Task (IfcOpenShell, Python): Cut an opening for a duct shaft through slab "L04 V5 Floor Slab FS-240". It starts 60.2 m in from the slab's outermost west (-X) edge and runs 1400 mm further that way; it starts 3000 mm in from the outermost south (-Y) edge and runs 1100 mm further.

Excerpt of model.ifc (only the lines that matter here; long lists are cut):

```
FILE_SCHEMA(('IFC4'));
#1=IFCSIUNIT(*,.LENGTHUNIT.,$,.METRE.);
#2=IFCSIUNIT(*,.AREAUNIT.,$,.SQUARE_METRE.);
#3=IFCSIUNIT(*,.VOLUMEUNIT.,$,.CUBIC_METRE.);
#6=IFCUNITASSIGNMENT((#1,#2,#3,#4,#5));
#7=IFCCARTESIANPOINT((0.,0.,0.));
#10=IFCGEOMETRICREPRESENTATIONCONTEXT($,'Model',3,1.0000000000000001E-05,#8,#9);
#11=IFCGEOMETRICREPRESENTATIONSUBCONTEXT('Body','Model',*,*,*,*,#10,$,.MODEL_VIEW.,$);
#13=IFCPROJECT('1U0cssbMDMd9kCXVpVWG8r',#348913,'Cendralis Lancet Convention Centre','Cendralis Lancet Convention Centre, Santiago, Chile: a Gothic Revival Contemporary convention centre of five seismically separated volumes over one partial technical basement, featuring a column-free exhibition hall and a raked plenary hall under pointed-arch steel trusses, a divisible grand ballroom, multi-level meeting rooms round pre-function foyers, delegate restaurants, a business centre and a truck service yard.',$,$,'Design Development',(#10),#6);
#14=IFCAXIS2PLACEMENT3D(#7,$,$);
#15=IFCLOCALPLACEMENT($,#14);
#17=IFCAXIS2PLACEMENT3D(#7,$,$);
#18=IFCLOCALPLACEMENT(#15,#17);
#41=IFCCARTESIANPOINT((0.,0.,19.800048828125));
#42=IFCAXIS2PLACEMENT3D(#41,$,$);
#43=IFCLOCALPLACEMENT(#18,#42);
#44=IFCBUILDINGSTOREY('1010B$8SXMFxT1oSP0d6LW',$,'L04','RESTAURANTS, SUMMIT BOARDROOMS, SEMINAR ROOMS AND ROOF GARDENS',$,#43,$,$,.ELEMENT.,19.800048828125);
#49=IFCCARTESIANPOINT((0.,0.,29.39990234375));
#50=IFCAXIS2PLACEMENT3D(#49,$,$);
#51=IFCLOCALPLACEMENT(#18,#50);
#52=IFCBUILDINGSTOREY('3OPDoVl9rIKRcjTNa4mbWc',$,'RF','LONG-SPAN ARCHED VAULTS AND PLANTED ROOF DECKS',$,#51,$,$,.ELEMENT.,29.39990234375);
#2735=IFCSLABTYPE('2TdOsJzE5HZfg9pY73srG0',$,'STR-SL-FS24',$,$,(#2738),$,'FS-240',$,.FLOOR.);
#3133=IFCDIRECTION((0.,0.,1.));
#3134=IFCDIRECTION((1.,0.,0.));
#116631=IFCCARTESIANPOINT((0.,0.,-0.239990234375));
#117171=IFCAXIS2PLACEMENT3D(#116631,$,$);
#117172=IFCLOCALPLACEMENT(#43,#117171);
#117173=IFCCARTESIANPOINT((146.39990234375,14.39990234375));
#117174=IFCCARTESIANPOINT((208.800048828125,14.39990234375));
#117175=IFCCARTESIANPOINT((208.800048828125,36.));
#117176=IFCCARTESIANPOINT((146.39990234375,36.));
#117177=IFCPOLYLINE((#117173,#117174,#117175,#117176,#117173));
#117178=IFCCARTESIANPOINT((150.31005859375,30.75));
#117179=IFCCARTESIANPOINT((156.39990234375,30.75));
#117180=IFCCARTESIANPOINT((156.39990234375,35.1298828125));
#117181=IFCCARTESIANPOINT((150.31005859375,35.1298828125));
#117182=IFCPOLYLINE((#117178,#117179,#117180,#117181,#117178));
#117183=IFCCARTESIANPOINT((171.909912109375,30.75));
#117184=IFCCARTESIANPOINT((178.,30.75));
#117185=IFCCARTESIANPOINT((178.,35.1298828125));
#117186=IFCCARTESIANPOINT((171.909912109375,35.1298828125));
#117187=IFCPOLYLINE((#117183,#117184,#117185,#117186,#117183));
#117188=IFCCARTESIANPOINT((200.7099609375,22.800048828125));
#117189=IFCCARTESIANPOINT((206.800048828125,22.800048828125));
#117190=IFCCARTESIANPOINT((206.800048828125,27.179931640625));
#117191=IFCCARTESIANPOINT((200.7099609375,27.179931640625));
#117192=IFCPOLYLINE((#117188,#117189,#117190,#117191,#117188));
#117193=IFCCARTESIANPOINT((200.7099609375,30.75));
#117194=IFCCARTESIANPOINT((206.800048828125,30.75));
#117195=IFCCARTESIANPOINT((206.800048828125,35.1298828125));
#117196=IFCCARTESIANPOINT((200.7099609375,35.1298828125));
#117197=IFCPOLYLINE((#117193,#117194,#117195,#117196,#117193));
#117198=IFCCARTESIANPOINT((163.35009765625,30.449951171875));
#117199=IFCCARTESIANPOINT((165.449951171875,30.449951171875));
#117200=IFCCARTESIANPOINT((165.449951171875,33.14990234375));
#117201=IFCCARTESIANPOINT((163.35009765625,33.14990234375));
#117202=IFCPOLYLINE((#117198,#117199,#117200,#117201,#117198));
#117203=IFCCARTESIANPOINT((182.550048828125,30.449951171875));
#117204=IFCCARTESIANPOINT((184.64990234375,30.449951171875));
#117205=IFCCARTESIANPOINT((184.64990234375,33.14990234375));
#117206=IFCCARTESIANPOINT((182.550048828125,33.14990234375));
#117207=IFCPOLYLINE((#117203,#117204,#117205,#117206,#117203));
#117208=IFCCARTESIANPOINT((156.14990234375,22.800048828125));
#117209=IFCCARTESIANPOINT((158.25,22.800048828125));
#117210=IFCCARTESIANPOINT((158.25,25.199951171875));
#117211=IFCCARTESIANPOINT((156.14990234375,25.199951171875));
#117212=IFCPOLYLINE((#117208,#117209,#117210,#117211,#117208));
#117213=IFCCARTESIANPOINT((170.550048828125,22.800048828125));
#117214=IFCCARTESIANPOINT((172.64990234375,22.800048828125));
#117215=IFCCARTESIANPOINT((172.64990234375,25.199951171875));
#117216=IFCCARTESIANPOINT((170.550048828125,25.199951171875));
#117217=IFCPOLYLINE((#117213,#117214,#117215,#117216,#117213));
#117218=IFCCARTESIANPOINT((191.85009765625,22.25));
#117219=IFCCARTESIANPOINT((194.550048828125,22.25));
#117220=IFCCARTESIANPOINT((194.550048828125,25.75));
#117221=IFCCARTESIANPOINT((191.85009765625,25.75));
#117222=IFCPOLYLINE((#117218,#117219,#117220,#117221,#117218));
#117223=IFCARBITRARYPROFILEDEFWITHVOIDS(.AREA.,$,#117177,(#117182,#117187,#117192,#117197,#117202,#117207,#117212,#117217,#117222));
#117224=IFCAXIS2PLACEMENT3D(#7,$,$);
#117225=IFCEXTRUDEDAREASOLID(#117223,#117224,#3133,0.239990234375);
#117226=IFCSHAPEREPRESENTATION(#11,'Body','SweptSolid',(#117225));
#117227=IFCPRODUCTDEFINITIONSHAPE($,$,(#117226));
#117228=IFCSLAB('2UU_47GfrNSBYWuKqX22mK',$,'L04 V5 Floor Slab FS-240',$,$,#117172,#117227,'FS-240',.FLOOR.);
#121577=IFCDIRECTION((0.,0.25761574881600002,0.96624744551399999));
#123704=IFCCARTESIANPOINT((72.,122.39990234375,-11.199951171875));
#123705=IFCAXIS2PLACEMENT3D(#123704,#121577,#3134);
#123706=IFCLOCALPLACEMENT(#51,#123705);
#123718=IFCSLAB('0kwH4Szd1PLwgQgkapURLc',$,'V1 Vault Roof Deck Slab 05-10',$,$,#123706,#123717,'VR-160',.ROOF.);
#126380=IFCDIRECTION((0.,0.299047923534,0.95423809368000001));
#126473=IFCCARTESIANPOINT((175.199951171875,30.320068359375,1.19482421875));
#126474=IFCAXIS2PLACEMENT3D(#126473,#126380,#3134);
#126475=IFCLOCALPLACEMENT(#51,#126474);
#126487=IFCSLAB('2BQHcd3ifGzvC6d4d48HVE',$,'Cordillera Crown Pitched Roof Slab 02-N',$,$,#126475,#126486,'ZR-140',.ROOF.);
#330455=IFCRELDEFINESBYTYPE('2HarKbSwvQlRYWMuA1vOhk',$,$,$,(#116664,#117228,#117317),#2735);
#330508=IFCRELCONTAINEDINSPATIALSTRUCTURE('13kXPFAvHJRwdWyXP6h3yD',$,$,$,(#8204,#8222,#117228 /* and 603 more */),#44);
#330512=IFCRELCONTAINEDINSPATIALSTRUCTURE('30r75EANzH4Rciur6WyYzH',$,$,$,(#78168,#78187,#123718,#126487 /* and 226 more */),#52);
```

```python
import numpy as np
import ifcopenshell
import ifcopenshell.api.feature
import ifcopenshell.api.geometry
import ifcopenshell.api.root
import ifcopenshell.geom
import ifcopenshell.util.placement
import ifcopenshell.util.representation
import ifcopenshell.util.shape
import ifcopenshell.util.unit

model = ifcopenshell.open("model.ifc")
unit_scale = ifcopenshell.util.unit.calculate_unit_scale(model)
settings = ifcopenshell.geom.settings()


def volume(element):
    """Net volume in cubic metres, openings subtracted."""
    shape = ifcopenshell.geom.create_shape(settings, element)
    return ifcopenshell.util.shape.get_volume(shape.geometry)


slab = model.by_guid("2UU_47GfrNSBYWuKqX22mK")
before = volume(slab)

# Extent in the slab's own axes, in metres. The edges named are its -X and -Y sides.
slab_shape = ifcopenshell.geom.create_shape(settings, slab)
vertices = ifcopenshell.util.shape.get_vertices(slab_shape.geometry)
x_min, y_min, bottom = vertices.min(axis=0)
top = vertices[:, 2].max()

opening = ifcopenshell.api.root.create_entity(model, ifc_class="IfcOpeningElement", name="Duct shaft opening", predefined_type="OPENING")
context = ifcopenshell.util.representation.get_context(model, "Model", "Body", "MODEL_VIEW")
width, depth = 1.4, 1.1
outline = [(0.0, 0.0), (width, 0.0), (width, depth), (0.0, depth), (0.0, 0.0)]
# Overshoot both faces by 50 mm so the cut is clean.
shape = ifcopenshell.api.geometry.add_slab_representation(
    model, context=context, depth=top - bottom + 0.1, polyline=outline
)
ifcopenshell.api.geometry.assign_representation(model, product=opening, representation=shape)

matrix = ifcopenshell.util.placement.get_local_placement(slab.ObjectPlacement)
matrix[:, 3] = matrix @ np.append(np.array([x_min + 60.2, y_min + 3, bottom - 0.05]) / unit_scale, 1.0)
ifcopenshell.api.geometry.edit_object_placement(model, product=opening, matrix=matrix, is_si=False)
ifcopenshell.api.feature.add_feature(model, feature=opening, element=slab)

after = volume(slab)

print(f"slab volume {before:.3f} -> {after:.3f} m3")

model.write("model_edited.ifc")
```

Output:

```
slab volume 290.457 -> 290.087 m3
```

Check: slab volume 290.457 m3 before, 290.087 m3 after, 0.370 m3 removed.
